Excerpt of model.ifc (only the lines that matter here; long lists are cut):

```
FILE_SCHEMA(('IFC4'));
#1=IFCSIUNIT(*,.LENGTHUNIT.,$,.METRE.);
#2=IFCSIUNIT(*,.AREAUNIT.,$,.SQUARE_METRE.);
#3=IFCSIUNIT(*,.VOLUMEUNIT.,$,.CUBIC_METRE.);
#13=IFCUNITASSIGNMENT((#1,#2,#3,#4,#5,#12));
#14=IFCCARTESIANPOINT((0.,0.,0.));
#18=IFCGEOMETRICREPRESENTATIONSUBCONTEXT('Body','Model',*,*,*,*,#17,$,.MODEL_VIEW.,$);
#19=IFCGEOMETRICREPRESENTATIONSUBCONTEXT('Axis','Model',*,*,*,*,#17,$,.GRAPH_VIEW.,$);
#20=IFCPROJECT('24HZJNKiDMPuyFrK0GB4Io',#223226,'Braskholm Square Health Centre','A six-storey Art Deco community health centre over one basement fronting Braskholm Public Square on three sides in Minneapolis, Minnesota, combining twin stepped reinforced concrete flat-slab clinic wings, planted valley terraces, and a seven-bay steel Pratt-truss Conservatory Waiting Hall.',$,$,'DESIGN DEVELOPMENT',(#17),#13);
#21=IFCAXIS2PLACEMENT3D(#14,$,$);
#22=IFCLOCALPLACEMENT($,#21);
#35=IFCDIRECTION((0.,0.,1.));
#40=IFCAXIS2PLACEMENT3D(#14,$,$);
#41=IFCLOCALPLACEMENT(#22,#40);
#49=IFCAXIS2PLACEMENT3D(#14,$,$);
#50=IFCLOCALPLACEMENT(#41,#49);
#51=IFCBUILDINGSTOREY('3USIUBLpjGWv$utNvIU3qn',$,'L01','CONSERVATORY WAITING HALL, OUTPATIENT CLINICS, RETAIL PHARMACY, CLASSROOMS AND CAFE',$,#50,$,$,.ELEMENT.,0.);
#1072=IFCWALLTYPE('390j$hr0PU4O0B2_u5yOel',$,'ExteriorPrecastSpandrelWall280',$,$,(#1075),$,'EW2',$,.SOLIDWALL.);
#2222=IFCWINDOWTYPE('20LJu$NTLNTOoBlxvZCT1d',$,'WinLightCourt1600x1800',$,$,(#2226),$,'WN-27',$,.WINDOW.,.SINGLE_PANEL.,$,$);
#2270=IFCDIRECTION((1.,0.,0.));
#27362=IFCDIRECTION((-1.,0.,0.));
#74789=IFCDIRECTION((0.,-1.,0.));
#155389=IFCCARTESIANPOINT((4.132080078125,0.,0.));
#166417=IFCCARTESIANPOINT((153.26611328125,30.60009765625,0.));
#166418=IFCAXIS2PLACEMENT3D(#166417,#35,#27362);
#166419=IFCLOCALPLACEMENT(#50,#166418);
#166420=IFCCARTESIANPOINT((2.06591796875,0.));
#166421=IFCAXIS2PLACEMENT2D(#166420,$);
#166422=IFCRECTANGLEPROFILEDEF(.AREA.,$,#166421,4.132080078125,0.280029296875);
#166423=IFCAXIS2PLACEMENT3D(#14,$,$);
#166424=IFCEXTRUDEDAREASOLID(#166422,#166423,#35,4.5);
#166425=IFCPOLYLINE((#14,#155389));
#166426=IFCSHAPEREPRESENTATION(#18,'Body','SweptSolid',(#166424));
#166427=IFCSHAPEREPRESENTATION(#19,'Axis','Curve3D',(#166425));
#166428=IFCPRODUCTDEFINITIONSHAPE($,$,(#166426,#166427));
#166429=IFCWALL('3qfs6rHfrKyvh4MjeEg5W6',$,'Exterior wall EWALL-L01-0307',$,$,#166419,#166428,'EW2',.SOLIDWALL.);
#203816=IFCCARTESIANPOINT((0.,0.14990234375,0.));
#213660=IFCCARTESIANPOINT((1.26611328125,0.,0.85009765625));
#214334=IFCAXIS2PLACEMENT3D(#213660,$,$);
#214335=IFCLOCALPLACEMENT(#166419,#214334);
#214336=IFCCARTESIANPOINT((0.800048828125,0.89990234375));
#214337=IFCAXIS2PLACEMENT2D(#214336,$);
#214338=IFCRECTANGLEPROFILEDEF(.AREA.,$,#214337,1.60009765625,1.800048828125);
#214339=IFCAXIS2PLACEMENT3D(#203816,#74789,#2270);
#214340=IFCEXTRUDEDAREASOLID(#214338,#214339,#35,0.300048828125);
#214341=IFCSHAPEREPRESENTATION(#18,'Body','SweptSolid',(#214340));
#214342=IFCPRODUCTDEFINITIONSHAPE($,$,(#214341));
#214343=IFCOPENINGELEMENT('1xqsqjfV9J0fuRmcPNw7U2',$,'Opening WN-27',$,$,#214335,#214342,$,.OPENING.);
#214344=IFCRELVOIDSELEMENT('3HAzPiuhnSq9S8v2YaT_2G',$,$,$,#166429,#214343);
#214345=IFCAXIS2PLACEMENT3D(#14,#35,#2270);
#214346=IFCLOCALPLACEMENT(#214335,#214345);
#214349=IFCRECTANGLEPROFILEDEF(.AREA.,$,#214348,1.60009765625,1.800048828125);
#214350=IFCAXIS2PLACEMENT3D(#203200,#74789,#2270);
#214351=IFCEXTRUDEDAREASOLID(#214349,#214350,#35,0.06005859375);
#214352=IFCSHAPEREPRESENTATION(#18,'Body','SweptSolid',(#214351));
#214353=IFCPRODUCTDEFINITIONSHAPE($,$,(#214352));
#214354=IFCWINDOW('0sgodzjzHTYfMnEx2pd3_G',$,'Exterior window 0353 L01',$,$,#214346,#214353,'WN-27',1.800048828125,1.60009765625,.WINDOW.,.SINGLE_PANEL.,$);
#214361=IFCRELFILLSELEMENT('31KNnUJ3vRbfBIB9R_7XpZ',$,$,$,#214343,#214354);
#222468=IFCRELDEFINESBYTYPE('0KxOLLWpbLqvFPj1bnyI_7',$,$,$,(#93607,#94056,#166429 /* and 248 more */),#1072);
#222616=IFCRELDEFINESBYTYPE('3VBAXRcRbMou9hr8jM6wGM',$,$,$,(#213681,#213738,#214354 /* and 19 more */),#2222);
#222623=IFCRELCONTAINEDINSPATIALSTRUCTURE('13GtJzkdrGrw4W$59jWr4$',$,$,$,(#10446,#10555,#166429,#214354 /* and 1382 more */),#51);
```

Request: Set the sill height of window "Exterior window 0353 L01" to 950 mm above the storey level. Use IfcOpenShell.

```python
import numpy as np
import ifcopenshell
import ifcopenshell.api.geometry
import ifcopenshell.geom
import ifcopenshell.util.element
import ifcopenshell.util.placement
import ifcopenshell.util.shape
import ifcopenshell.util.unit

model = ifcopenshell.open("model.ifc")
unit_scale = ifcopenshell.util.unit.calculate_unit_scale(model)

window = model.by_id(214354)
opening = window.FillsVoids[0].RelatingOpeningElement
storey = ifcopenshell.util.element.get_container(window, ifc_class="IfcBuildingStorey")
level = ifcopenshell.util.placement.get_local_placement(storey.ObjectPlacement)[2, 3]

# The opening's origin need not be at the sill, so measure its lowest point.
shape = ifcopenshell.geom.create_shape(ifcopenshell.geom.settings(), opening)
bottom = ifcopenshell.util.shape.get_shape_bottom_elevation(shape, shape.geometry) / unit_scale
dz = level + 0.95 - bottom

shift = np.array([0.0, 0.0, dz])
# The window is placed relative to its opening, so it follows when the opening moves.
matrix = ifcopenshell.util.placement.get_local_placement(opening.ObjectPlacement)
matrix[:3, 3] += shift
ifcopenshell.api.geometry.edit_object_placement(
    model, product=opening, matrix=matrix, is_si=False, should_transform_children=True
)

print(f"moved by {dz * unit_scale:+.3f} m")

model.write("model_updated.ifc")
```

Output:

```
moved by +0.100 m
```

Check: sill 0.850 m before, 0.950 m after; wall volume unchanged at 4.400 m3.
